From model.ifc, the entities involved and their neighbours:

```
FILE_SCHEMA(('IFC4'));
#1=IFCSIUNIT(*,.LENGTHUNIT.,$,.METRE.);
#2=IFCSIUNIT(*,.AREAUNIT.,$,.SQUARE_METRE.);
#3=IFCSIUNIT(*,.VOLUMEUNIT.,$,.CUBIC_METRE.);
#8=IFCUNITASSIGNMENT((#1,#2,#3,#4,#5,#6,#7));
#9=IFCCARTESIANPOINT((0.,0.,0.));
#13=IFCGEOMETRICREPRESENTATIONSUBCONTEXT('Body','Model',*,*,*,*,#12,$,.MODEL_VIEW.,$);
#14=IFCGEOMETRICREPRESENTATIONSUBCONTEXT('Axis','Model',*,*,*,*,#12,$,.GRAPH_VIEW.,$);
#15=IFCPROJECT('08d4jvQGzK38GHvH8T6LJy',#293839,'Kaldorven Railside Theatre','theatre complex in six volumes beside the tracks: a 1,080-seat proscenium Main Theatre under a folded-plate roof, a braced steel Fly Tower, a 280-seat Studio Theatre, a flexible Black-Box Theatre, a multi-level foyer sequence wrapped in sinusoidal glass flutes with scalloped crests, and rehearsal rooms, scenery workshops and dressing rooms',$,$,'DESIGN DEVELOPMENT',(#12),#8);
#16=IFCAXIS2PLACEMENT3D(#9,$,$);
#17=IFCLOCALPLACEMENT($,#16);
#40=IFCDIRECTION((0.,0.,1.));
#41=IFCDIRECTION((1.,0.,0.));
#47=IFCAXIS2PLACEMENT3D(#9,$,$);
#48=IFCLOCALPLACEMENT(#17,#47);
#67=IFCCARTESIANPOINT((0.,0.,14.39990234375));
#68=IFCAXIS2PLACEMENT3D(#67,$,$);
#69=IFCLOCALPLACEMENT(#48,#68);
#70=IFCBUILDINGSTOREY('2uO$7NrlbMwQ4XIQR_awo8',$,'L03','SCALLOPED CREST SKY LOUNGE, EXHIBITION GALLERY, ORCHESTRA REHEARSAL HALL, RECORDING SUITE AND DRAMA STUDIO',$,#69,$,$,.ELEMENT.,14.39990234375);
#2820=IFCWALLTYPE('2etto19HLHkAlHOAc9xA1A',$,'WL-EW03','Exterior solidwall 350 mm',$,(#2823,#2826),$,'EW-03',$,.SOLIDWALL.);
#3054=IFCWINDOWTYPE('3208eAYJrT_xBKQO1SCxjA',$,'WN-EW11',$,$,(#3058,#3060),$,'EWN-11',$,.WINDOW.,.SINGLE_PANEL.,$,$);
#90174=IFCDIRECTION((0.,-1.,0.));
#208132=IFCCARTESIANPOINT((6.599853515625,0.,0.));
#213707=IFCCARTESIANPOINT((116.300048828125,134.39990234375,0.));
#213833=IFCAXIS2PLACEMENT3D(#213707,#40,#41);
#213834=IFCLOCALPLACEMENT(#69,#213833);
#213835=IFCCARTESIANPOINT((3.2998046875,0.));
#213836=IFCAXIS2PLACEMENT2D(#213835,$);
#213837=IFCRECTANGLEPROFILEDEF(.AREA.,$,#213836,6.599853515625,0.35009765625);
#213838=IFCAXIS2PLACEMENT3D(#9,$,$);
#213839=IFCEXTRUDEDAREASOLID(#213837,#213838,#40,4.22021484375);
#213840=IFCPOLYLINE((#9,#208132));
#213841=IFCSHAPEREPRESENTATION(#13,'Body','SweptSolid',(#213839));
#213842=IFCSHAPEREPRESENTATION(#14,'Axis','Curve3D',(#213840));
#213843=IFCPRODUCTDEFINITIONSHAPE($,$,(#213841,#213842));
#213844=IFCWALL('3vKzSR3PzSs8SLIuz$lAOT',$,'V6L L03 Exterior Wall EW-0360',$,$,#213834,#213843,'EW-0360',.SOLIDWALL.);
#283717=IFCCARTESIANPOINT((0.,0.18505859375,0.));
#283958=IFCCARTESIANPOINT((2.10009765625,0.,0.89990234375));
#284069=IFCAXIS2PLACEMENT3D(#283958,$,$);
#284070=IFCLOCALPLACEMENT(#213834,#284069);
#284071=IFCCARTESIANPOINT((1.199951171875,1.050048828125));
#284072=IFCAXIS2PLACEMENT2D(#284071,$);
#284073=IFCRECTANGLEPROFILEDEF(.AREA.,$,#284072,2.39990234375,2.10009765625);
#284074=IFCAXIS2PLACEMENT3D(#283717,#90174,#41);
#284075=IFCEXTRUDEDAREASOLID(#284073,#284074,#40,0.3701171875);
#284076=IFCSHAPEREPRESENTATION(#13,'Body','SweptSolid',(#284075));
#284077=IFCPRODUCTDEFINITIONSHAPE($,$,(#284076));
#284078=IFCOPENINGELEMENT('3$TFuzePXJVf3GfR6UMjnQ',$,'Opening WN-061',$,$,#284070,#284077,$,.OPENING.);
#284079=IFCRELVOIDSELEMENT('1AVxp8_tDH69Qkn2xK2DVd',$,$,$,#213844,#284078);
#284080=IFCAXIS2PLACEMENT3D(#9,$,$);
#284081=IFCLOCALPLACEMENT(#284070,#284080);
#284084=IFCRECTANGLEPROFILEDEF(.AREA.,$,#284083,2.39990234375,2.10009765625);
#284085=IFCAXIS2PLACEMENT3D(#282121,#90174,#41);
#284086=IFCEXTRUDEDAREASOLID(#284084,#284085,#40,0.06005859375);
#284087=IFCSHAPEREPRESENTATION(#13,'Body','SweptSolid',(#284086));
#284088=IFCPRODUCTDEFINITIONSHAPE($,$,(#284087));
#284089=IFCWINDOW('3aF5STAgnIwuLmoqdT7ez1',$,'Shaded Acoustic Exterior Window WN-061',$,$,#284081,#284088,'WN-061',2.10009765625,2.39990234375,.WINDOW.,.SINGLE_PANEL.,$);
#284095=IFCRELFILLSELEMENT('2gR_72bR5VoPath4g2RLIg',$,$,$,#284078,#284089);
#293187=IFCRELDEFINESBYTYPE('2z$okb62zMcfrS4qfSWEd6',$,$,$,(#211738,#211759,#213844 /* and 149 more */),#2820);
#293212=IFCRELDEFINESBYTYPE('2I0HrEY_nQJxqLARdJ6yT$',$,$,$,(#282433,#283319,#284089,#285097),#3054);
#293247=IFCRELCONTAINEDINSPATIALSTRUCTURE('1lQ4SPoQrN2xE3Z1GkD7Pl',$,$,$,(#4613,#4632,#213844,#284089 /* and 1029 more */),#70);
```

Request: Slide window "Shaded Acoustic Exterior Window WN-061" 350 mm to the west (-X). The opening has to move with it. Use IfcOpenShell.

```python
import ifcopenshell
import ifcopenshell.api.geometry
import ifcopenshell.util.placement

model = ifcopenshell.open("model.ifc")

window = model.by_guid("3aF5STAgnIwuLmoqdT7ez1")
opening = window.FillsVoids[0].RelatingOpeningElement
wall = opening.VoidsElements[0].RelatingBuildingElement

wall_matrix = ifcopenshell.util.placement.get_local_placement(wall.ObjectPlacement)
shift = wall_matrix[:3, 0] * -0.35
before = ifcopenshell.util.placement.get_local_placement(window.ObjectPlacement)[:3, 3].copy()

# The window is placed relative to its opening, so it follows when the opening moves.
matrix = ifcopenshell.util.placement.get_local_placement(opening.ObjectPlacement)
matrix[:3, 3] += shift
ifcopenshell.api.geometry.edit_object_placement(
    model, product=opening, matrix=matrix, is_si=False, should_transform_children=True
)

after = ifcopenshell.util.placement.get_local_placement(window.ObjectPlacement)[:3, 3]
print("window moved by", (after - before).round(3) + 0.0)

model.write("model_rev.ifc")
```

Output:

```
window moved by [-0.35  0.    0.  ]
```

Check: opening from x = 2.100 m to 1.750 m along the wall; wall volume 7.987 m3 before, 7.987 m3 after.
